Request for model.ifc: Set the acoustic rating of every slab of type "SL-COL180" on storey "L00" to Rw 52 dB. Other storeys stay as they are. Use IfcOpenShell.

First a look at what the model holds.

```python
import ifcopenshell
import ifcopenshell.util.element

model = ifcopenshell.open("model.ifc")
print(model.schema)
storey = next(s for s in model.by_type("IfcBuildingStorey") if s.Name == "L00")
slabs = [e for e in ifcopenshell.util.element.get_decomposition(storey) if e.is_a("IfcSlab")]
seen = {}
for e in slabs:
    element_type = ifcopenshell.util.element.get_type(e)
    key = (element_type.Name if element_type != e and element_type else None, ifcopenshell.util.element.get_pset(e, "Pset_SlabCommon", "AcousticRating"))
    seen[key] = seen.get(key, 0) + 1
for (name, value), count in sorted(seen.items(), key=str):
    print(count, "x", name, "|", value)
```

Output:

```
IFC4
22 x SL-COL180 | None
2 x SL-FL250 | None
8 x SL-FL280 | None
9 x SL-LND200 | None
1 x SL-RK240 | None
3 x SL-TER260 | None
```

```python
import ifcopenshell
import ifcopenshell.api.pset
import ifcopenshell.util.element

model = ifcopenshell.open("model.ifc")

storey = next(s for s in model.by_type("IfcBuildingStorey") if s.Name == "L00")
slabs = [e for e in ifcopenshell.util.element.get_decomposition(storey) if e.is_a("IfcSlab")]

count = 0
for e in slabs:
    element_type = ifcopenshell.util.element.get_type(e)
    if element_type in (None, e) or element_type.Name != "SL-COL180":
        continue
    # add_pset returns the element's existing set when there is one.
    pset = ifcopenshell.api.pset.add_pset(model, product=e, name="Pset_SlabCommon")
    ifcopenshell.api.pset.edit_pset(model, pset=pset, properties={"AcousticRating": "Rw 52 dB"})
    count += 1

print(count, "slabs updated")

model.write("model_v2.ifc")
```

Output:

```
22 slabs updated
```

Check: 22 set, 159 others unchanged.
